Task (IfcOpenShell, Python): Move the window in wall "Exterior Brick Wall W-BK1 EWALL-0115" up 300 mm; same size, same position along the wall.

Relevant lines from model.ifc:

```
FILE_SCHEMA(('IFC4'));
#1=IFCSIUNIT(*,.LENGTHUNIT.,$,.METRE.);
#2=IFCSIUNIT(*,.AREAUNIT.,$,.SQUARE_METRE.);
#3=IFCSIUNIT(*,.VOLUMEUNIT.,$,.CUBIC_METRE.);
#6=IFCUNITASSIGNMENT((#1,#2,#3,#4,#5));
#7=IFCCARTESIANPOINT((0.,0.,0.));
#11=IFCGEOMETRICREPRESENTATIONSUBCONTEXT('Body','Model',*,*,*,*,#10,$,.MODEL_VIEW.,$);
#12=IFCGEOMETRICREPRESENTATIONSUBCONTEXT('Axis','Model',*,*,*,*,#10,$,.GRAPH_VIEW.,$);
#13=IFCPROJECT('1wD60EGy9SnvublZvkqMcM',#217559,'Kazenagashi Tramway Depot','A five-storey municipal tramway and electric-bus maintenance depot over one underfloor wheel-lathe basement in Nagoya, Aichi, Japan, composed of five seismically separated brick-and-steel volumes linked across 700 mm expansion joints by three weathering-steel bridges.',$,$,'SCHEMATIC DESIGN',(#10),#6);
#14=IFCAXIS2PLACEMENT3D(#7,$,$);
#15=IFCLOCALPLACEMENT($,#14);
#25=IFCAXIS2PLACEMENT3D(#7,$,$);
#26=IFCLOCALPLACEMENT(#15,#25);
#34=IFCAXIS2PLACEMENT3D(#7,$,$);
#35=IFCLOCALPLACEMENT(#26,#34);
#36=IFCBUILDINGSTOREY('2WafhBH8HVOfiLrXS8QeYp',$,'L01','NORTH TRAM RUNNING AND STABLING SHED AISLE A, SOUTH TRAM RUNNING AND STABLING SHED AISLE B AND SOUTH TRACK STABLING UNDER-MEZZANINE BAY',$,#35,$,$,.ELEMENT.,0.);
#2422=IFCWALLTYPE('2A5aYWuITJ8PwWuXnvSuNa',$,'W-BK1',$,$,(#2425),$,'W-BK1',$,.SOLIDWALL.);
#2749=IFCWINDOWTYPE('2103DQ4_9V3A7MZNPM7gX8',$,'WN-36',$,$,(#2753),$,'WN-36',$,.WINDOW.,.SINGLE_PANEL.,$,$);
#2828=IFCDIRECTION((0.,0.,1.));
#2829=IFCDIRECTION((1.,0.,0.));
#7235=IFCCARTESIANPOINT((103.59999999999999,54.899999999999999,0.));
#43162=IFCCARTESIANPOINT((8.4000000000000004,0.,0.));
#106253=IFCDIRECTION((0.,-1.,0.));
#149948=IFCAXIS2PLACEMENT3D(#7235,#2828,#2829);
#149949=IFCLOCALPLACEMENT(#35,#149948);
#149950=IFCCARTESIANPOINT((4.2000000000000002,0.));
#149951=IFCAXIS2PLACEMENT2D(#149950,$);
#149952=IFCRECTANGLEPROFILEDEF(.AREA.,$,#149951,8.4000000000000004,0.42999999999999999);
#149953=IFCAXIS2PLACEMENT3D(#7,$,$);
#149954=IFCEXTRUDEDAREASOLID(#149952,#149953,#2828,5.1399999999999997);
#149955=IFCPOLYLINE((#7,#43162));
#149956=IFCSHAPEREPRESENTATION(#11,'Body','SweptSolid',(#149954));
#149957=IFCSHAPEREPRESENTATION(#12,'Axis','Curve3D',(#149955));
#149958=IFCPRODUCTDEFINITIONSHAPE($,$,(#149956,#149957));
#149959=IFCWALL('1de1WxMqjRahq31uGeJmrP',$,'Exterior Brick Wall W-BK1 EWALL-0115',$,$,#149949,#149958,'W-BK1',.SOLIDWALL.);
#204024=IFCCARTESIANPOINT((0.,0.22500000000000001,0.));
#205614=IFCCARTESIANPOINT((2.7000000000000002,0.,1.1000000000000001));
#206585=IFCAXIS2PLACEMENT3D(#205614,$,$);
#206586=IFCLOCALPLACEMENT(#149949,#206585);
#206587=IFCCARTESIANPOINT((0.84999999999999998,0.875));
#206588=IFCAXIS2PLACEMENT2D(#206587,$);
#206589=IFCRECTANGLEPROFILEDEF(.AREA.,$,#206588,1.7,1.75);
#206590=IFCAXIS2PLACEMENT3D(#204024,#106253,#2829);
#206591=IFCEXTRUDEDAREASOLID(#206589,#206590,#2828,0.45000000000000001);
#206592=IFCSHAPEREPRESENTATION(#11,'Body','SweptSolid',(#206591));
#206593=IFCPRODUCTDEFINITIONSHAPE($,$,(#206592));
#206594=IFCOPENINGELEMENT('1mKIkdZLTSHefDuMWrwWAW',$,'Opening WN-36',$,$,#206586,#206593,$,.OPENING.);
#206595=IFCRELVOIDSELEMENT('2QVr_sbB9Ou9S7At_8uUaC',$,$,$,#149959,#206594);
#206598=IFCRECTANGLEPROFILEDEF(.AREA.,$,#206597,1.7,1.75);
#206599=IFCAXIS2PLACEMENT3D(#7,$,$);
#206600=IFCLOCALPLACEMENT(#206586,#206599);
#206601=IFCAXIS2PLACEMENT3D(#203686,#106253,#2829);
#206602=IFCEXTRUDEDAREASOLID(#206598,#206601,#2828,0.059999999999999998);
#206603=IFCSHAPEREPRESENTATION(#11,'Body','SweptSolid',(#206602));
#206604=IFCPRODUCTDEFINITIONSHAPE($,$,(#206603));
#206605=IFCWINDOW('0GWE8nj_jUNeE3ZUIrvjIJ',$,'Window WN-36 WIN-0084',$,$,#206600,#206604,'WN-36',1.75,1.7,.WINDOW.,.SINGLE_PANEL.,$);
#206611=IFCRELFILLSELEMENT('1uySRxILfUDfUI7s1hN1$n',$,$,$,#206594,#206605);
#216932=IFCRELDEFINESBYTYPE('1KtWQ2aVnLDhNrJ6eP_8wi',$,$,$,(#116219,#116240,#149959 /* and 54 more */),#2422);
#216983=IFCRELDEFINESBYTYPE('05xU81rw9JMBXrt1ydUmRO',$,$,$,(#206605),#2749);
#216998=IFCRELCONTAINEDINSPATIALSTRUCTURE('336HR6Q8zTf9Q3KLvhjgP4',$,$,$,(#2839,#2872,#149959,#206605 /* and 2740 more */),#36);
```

```python
import numpy as np
import ifcopenshell
import ifcopenshell.api.geometry
import ifcopenshell.util.placement
import ifcopenshell.util.unit

model = ifcopenshell.open("model.ifc")
unit_scale = ifcopenshell.util.unit.calculate_unit_scale(model)

window = model.by_id(206605)
opening = window.FillsVoids[0].RelatingOpeningElement
dz = 0.3 / unit_scale

shift = np.array([0.0, 0.0, dz])
# The window is placed relative to its opening, so it follows when the opening moves.
matrix = ifcopenshell.util.placement.get_local_placement(opening.ObjectPlacement)
matrix[:3, 3] += shift
ifcopenshell.api.geometry.edit_object_placement(
    model, product=opening, matrix=matrix, is_si=False, should_transform_children=True
)

print(f"moved by {dz * unit_scale:+.3f} m")

model.write("model_rev.ifc")
```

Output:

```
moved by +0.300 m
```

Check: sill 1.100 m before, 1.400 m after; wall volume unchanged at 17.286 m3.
